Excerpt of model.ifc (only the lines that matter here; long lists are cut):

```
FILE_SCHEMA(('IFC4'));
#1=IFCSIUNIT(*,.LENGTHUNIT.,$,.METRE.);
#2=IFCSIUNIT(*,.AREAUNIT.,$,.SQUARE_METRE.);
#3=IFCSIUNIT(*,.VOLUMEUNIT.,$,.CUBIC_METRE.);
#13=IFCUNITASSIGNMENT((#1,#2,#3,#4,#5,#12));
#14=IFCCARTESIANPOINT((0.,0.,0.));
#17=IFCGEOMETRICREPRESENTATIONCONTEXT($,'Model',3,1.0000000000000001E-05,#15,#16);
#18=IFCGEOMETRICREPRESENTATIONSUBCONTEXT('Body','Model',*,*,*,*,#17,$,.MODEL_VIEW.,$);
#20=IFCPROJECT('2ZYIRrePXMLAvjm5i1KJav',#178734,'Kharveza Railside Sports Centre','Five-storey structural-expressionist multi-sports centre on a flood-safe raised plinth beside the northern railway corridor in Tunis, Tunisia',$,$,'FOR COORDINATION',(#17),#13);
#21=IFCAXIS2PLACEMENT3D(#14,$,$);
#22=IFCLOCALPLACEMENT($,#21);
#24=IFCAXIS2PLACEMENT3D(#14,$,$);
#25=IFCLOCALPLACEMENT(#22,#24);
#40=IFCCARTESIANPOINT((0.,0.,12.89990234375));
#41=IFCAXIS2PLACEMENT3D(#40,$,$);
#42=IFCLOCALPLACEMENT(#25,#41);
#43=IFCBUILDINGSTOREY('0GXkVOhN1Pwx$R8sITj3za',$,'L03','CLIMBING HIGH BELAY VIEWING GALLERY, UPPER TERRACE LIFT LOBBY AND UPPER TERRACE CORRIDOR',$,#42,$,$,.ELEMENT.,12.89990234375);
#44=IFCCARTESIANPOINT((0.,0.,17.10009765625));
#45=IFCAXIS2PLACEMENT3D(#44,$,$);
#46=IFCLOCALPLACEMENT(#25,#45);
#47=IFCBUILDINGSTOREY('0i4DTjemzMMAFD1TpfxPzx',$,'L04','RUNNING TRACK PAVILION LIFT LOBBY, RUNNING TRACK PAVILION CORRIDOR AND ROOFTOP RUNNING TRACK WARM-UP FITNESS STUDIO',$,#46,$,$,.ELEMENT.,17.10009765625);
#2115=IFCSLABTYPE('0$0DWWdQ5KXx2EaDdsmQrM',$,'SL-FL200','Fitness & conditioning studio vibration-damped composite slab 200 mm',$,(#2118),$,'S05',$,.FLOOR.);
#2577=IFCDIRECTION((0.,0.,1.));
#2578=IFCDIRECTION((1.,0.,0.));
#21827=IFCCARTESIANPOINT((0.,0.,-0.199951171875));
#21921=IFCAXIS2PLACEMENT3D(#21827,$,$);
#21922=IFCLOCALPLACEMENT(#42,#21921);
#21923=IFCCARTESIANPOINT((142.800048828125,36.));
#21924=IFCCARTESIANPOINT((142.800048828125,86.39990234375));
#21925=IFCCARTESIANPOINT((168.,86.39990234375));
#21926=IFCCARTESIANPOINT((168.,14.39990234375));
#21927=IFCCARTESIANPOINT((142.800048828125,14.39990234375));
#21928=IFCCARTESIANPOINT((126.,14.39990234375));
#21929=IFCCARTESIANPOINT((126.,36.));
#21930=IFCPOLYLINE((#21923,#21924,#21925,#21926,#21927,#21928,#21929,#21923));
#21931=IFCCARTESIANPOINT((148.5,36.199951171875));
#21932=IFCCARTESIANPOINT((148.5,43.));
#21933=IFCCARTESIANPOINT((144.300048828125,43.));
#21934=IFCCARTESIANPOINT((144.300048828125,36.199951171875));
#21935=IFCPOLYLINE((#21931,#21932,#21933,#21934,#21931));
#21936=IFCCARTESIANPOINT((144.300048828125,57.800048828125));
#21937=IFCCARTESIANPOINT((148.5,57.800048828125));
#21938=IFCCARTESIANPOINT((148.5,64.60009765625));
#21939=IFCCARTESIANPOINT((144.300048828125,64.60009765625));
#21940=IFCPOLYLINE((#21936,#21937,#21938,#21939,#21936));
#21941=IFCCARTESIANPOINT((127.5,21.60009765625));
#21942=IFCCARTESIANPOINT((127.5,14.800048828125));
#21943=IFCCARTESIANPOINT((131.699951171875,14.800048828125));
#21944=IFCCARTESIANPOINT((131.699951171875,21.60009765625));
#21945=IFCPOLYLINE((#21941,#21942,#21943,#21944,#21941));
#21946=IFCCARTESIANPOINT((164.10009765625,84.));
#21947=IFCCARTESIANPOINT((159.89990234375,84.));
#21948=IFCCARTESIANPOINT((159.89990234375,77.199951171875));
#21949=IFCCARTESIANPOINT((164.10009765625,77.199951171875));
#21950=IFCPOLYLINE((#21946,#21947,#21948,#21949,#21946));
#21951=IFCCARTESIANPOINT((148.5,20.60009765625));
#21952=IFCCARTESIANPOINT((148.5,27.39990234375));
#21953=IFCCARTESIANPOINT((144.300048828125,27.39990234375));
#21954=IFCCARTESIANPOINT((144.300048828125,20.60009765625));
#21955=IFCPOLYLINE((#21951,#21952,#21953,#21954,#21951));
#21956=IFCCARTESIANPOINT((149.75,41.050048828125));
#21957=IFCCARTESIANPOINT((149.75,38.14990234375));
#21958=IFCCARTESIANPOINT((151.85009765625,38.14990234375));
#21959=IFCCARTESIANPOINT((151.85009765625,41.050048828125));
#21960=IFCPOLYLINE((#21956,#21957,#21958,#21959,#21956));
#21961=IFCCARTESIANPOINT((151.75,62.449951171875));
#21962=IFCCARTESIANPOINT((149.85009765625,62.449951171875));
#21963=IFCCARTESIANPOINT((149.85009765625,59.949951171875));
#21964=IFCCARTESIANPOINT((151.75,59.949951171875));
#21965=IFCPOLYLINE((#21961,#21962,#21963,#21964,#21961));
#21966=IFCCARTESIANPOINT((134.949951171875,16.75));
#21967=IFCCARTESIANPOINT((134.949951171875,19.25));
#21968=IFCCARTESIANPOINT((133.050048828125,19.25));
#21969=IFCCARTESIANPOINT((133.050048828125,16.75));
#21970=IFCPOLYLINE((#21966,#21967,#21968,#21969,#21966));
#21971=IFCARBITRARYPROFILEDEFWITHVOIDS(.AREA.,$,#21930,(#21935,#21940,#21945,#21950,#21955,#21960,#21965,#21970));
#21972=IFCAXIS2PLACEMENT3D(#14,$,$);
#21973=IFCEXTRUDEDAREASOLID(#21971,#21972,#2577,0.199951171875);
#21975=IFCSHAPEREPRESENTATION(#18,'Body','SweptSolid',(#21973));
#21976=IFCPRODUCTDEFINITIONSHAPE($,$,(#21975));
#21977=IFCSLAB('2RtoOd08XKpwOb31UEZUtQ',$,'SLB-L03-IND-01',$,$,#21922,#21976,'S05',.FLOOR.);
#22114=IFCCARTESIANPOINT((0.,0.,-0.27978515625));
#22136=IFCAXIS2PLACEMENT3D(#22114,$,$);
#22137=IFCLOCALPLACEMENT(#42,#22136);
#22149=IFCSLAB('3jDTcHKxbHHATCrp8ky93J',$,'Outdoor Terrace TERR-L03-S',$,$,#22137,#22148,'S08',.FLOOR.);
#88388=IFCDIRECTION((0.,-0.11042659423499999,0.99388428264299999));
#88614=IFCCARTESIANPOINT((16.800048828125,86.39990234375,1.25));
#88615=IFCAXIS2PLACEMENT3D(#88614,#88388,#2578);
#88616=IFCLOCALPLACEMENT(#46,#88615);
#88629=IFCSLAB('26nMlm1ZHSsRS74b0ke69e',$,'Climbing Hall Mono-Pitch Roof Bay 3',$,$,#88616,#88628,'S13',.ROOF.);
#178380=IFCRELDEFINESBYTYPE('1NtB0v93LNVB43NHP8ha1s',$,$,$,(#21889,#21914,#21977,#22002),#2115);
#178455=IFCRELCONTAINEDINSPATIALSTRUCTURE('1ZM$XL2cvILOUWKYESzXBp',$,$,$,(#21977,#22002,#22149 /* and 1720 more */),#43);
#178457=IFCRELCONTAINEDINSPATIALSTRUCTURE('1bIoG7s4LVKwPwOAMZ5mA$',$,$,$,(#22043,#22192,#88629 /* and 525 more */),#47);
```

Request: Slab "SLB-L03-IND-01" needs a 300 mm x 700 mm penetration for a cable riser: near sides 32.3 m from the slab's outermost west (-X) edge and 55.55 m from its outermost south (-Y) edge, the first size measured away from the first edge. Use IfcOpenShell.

```python
import numpy as np
import ifcopenshell
import ifcopenshell.api.feature
import ifcopenshell.api.geometry
import ifcopenshell.api.root
import ifcopenshell.geom
import ifcopenshell.util.placement
import ifcopenshell.util.representation
import ifcopenshell.util.shape
import ifcopenshell.util.unit

model = ifcopenshell.open("model.ifc")
unit_scale = ifcopenshell.util.unit.calculate_unit_scale(model)
settings = ifcopenshell.geom.settings()


def volume(element):
    """Net volume in cubic metres, openings subtracted."""
    shape = ifcopenshell.geom.create_shape(settings, element)
    return ifcopenshell.util.shape.get_volume(shape.geometry)


slab = model.by_guid("2RtoOd08XKpwOb31UEZUtQ")
before = volume(slab)

# Extent in the slab's own axes, in metres. The edges named are its -X and -Y sides.
slab_shape = ifcopenshell.geom.create_shape(settings, slab)
vertices = ifcopenshell.util.shape.get_vertices(slab_shape.geometry)
x_min, y_min, bottom = vertices.min(axis=0)
top = vertices[:, 2].max()

opening = ifcopenshell.api.root.create_entity(model, ifc_class="IfcOpeningElement", name="Cable riser opening", predefined_type="OPENING")
context = ifcopenshell.util.representation.get_context(model, "Model", "Body", "MODEL_VIEW")
width, depth = 0.3, 0.7
outline = [(0.0, 0.0), (width, 0.0), (width, depth), (0.0, depth), (0.0, 0.0)]
# Overshoot both faces by 50 mm so the cut is clean.
shape = ifcopenshell.api.geometry.add_slab_representation(
    model, context=context, depth=top - bottom + 0.1, polyline=outline
)
ifcopenshell.api.geometry.assign_representation(model, product=opening, representation=shape)

matrix = ifcopenshell.util.placement.get_local_placement(slab.ObjectPlacement)
matrix[:, 3] = matrix @ np.append(np.array([x_min + 32.3, y_min + 55.55, bottom - 0.05]) / unit_scale, 1.0)
ifcopenshell.api.geometry.edit_object_placement(model, product=opening, matrix=matrix, is_si=False)
ifcopenshell.api.feature.add_feature(model, feature=opening, element=slab)

after = volume(slab)

print(f"slab volume {before:.3f} -> {after:.3f} m3")

model.write("model-out.ifc")
```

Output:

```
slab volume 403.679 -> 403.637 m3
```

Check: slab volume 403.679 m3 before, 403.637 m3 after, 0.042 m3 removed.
